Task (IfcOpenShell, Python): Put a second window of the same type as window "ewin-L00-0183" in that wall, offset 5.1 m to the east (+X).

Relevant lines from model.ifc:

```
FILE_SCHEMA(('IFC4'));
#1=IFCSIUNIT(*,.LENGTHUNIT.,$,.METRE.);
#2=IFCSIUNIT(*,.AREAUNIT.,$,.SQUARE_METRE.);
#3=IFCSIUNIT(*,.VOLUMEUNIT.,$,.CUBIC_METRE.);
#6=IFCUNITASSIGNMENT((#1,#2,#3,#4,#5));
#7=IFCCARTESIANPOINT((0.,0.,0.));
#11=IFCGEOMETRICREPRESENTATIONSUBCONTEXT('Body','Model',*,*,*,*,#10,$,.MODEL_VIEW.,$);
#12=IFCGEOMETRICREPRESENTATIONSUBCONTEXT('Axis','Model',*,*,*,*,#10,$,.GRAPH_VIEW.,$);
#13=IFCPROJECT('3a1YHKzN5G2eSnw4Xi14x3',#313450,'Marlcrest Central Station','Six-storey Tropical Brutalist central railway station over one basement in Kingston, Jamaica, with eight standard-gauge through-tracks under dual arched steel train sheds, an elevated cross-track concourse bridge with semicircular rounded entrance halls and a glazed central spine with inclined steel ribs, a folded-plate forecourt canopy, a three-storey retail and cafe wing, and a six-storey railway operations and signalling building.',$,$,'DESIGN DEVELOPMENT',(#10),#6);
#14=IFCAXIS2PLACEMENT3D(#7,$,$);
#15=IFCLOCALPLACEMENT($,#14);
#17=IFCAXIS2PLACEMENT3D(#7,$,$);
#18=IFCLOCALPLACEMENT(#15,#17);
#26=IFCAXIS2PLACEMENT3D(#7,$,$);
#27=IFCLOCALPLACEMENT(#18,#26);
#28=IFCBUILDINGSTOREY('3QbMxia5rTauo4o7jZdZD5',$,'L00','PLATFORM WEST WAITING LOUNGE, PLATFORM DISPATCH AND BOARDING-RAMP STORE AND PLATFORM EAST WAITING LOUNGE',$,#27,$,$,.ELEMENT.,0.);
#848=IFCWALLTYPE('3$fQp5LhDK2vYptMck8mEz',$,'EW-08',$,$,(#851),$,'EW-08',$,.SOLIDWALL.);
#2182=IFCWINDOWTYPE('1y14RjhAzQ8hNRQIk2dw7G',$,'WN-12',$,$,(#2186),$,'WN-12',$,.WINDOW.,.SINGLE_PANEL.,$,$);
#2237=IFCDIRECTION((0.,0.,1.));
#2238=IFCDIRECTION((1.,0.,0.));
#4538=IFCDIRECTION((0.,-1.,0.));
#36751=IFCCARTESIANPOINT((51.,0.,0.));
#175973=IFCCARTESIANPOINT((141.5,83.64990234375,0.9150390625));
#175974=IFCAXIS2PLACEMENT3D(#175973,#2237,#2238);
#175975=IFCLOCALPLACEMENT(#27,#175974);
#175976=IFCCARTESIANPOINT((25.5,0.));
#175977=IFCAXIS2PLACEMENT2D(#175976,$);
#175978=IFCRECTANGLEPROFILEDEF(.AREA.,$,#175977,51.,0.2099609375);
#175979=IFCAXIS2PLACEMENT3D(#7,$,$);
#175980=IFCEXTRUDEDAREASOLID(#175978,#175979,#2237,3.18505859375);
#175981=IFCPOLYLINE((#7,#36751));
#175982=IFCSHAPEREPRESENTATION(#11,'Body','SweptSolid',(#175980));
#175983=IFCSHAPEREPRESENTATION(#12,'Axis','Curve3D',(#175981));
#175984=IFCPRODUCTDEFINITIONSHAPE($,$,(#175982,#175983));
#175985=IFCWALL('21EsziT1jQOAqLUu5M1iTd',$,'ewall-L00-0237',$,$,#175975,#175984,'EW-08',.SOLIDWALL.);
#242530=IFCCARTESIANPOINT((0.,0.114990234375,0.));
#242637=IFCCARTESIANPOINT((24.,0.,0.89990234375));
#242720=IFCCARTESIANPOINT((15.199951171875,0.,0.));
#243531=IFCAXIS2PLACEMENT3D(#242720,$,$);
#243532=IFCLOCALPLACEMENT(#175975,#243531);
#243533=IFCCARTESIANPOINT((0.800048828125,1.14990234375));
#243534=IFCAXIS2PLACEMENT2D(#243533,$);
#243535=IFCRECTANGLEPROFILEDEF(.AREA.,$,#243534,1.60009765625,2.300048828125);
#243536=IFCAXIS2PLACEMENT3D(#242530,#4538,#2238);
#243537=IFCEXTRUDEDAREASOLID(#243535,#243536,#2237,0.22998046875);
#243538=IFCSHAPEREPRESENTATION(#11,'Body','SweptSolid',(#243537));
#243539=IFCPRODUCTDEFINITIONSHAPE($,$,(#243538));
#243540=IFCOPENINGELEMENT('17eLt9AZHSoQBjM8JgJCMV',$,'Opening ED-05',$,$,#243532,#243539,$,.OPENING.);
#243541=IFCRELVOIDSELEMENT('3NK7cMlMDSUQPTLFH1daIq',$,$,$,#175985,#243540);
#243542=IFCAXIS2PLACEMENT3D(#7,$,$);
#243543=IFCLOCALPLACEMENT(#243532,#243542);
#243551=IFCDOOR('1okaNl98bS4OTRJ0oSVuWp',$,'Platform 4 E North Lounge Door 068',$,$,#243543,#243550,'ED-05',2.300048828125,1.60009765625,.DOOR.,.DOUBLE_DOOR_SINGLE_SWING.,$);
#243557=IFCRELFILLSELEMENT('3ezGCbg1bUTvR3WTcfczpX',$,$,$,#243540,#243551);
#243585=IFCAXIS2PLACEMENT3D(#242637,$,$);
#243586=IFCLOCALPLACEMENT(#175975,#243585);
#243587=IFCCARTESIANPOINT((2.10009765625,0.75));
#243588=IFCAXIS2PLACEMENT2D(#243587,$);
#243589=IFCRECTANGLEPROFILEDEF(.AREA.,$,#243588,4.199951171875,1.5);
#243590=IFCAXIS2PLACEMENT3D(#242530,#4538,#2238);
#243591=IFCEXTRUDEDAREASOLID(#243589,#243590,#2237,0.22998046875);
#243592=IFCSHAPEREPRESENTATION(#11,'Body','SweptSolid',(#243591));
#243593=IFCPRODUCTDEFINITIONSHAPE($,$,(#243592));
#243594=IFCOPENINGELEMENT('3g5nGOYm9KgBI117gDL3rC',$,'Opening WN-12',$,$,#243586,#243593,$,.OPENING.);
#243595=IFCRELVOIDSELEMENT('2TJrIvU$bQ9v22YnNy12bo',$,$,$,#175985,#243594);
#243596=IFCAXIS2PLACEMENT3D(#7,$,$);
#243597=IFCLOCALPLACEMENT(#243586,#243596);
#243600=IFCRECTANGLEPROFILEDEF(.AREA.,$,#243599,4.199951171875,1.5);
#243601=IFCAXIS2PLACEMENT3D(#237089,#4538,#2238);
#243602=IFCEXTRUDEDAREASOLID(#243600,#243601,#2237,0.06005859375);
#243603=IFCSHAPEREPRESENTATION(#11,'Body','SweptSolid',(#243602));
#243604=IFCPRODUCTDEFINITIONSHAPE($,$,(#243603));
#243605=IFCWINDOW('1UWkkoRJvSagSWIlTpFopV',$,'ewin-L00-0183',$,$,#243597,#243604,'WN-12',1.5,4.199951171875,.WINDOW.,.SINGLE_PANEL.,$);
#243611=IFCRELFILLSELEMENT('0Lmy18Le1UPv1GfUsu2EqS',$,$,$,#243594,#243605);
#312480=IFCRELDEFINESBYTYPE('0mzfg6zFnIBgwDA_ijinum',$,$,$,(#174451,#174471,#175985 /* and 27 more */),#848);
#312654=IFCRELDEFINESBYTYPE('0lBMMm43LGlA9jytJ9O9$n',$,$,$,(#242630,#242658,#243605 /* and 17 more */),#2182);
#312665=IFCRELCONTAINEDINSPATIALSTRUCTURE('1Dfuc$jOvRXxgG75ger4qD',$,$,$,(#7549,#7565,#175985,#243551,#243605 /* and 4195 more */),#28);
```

```python
import ifcopenshell
import ifcopenshell.api.feature
import ifcopenshell.api.geometry
import ifcopenshell.api.root
import ifcopenshell.geom
import ifcopenshell.util.element
import ifcopenshell.util.placement
import ifcopenshell.util.shape
import ifcopenshell.util.unit

model = ifcopenshell.open("model.ifc")
unit_scale = ifcopenshell.util.unit.calculate_unit_scale(model)
settings = ifcopenshell.geom.settings()


def volume(element):
    """Net volume in cubic metres, openings subtracted."""
    shape = ifcopenshell.geom.create_shape(settings, element)
    return ifcopenshell.util.shape.get_volume(shape.geometry)


window = model.by_guid("1UWkkoRJvSagSWIlTpFopV")
opening = window.FillsVoids[0].RelatingOpeningElement
wall = opening.VoidsElements[0].RelatingBuildingElement
before = volume(wall)
shift = ifcopenshell.util.placement.get_local_placement(wall.ObjectPlacement)[:3, 0] * 5.1 / unit_scale

# copy_class copies the void relationship, type, container and properties, but no geometry.
new_opening = ifcopenshell.api.root.copy_class(model, product=opening)
new_opening.Representation = ifcopenshell.util.element.copy_deep(
    model, opening.Representation, exclude=["IfcGeometricRepresentationContext", "IfcRepresentationMap"]
)
new_window = ifcopenshell.api.root.copy_class(model, product=window)
new_window.Representation = ifcopenshell.util.element.copy_deep(
    model, window.Representation, exclude=["IfcGeometricRepresentationContext", "IfcRepresentationMap"]
)
new_window.Tag = None
ifcopenshell.api.feature.add_filling(model, opening=new_opening, element=new_window)

for old, new in ((opening, new_opening), (window, new_window)):
    matrix = ifcopenshell.util.placement.get_local_placement(old.ObjectPlacement)
    matrix[:3, 3] += shift
    ifcopenshell.api.geometry.edit_object_placement(model, product=new, matrix=matrix, is_si=False)

after = volume(wall)

print(f"wall volume {before:.3f} -> {after:.3f} m3")

model.write("model_edited.ifc")
```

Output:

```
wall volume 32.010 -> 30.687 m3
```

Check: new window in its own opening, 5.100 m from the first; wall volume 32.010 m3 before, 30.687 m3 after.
